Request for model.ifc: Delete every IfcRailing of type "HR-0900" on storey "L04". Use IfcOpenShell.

First a look at what the model holds.

```python
import ifcopenshell
import ifcopenshell.util.element

model = ifcopenshell.open("model.ifc")
print(model.schema)
storey = next(s for s in model.by_type("IfcBuildingStorey") if s.Name == "L04")
railings = [e for e in ifcopenshell.util.element.get_decomposition(storey) if e.is_a("IfcRailing")]
seen = {}
for e in railings:
    element_type = ifcopenshell.util.element.get_type(e)
    name = element_type.Name if element_type not in (None, e) else None
    seen[name] = seen.get(name, 0) + 1
for name, count in sorted(seen.items(), key=str):
    print(count, "x", name)
```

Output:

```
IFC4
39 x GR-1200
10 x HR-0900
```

```python
import ifcopenshell
import ifcopenshell.api.root
import ifcopenshell.util.element

model = ifcopenshell.open("model.ifc")

storey = next(s for s in model.by_type("IfcBuildingStorey") if s.Name == "L04")
railings = [e for e in ifcopenshell.util.element.get_decomposition(storey) if e.is_a("IfcRailing")]
targets = [e for e in railings if (t := ifcopenshell.util.element.get_type(e)) not in (None, e) and t.Name == "HR-0900"]

for e in targets:
    ifcopenshell.api.root.remove_product(model, product=e)
print(len(targets), "removed")

model.write("model_rev.ifc")
```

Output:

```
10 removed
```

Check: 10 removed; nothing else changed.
